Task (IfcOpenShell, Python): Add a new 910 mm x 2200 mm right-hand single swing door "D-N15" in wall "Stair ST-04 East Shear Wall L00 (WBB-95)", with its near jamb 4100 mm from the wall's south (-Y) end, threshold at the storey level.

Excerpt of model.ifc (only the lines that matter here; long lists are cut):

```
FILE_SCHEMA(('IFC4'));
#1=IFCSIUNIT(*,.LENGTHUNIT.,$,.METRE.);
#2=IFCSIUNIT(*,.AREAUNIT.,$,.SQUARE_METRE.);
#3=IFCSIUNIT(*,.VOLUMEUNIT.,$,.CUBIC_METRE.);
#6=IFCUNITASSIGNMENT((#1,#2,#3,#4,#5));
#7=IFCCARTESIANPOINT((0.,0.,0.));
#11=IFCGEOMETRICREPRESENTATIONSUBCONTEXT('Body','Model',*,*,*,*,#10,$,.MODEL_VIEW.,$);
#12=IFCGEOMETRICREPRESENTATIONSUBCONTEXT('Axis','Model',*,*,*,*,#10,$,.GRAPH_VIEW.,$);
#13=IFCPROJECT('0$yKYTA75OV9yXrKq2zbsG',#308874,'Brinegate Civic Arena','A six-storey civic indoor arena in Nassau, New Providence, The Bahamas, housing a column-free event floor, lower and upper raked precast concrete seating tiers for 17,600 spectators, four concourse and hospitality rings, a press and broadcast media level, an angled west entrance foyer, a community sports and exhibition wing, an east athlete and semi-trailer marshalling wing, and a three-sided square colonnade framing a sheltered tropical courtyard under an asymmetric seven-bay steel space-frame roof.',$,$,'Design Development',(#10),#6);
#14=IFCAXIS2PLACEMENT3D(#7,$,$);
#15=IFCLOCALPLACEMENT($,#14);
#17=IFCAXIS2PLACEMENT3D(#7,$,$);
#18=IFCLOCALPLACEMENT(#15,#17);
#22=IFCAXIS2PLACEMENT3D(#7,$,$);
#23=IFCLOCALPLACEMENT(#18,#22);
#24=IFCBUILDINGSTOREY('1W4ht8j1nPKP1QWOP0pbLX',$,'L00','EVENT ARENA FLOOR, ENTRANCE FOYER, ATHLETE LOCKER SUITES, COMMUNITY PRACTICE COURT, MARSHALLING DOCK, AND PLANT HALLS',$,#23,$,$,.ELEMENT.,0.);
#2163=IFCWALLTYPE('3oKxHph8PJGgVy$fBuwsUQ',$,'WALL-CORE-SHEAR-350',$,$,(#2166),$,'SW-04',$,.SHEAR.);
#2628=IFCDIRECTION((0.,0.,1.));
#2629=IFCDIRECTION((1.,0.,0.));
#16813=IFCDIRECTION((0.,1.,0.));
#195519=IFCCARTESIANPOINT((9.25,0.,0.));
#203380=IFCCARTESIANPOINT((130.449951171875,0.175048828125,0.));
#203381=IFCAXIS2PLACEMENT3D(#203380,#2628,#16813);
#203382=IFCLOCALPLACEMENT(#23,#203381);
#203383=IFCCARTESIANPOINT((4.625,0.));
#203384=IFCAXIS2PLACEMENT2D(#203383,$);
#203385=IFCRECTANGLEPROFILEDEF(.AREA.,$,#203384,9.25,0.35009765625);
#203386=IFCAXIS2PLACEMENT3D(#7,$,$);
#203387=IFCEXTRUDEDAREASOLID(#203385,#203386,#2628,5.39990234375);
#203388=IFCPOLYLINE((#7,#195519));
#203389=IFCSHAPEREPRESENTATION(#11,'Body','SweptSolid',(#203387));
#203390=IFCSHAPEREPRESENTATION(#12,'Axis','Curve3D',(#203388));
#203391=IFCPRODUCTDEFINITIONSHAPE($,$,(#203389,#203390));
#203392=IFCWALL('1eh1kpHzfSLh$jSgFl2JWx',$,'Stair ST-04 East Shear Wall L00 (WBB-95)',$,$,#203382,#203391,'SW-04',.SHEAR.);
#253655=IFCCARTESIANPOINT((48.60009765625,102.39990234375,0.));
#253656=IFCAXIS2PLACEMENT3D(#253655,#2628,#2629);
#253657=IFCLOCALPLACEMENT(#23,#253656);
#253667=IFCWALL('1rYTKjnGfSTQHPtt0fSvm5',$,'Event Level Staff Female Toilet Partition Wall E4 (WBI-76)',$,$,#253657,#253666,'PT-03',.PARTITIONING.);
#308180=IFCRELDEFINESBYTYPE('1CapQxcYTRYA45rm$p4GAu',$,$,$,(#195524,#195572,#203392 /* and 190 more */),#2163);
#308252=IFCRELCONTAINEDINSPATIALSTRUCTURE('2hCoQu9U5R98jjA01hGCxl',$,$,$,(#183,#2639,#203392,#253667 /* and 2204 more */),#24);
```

```python
import numpy as np
import ifcopenshell
import ifcopenshell.api.feature
import ifcopenshell.api.geometry
import ifcopenshell.api.root
import ifcopenshell.api.spatial
import ifcopenshell.geom
import ifcopenshell.util.element
import ifcopenshell.util.placement
import ifcopenshell.util.representation
import ifcopenshell.util.shape
import ifcopenshell.util.unit

model = ifcopenshell.open("model.ifc")
unit_scale = ifcopenshell.util.unit.calculate_unit_scale(model)
settings = ifcopenshell.geom.settings()


def volume(element):
    """Net volume in cubic metres, openings subtracted."""
    shape = ifcopenshell.geom.create_shape(settings, element)
    return ifcopenshell.util.shape.get_volume(shape.geometry)


wall = model.by_guid("1eh1kpHzfSLh$jSgFl2JWx")
storey = ifcopenshell.util.element.get_container(wall, ifc_class="IfcBuildingStorey")
context = ifcopenshell.util.representation.get_context(model, "Model", "Body", "MODEL_VIEW")
before = volume(wall)

width, height, from_end, sill = 0.91, 2.2, 4.1, 0.0  # metres

# The wall runs along its own X axis, and the end named is its -X end.
wall_shape = ifcopenshell.geom.create_shape(settings, wall)
x, y, z = ifcopenshell.util.shape.get_vertices(wall_shape.geometry).T
start = x.min() + from_end
face, thickness = float(y.min()), float(y.max() - y.min())
wall_matrix = ifcopenshell.util.placement.get_local_placement(wall.ObjectPlacement)
level = ifcopenshell.util.placement.get_local_placement(storey.ObjectPlacement)[2, 3]


def in_wall(x, y):
    """Placement at x, y metres in the wall's axes, at sill height."""
    matrix = wall_matrix.copy()
    matrix[:, 3] = wall_matrix @ np.array([x / unit_scale, y / unit_scale, 0.0, 1.0])
    matrix[2, 3] = level + sill / unit_scale
    return matrix


# Opening: a box that overshoots both wall faces by 50 mm.
opening = ifcopenshell.api.root.create_entity(model, ifc_class="IfcOpeningElement", predefined_type="OPENING")
box = ifcopenshell.api.geometry.add_wall_representation(
    model, context=context, length=width, height=height, thickness=thickness + 0.1
)
ifcopenshell.api.geometry.assign_representation(model, product=opening, representation=box)
ifcopenshell.api.geometry.edit_object_placement(model, product=opening, matrix=in_wall(start, face - 0.05), is_si=False)
ifcopenshell.api.feature.add_feature(model, feature=opening, element=wall)

door = ifcopenshell.api.root.create_entity(model, ifc_class="IfcDoor", name="D-N15", predefined_type="DOOR")
door.OverallWidth, door.OverallHeight = width / unit_scale, height / unit_scale
door.OperationType = "SINGLE_SWING_RIGHT"
body = ifcopenshell.api.geometry.add_door_representation(
    model,
    context=context,
    overall_width=door.OverallWidth,
    overall_height=door.OverallHeight,
    operation_type="SINGLE_SWING_RIGHT",
    lining_properties={"LiningDepth": thickness / unit_scale, "ThresholdDepth": thickness / unit_scale},
)
ifcopenshell.api.geometry.assign_representation(model, product=door, representation=body)
ifcopenshell.api.spatial.assign_container(model, products=[door], relating_structure=storey)
ifcopenshell.api.feature.add_filling(model, opening=opening, element=door)

# The lining spans the wall, so the door starts at the wall face.
ifcopenshell.api.geometry.edit_object_placement(model, product=door, matrix=in_wall(start, face), is_si=False)

after = volume(wall)

print(f"wall volume {before:.3f} -> {after:.3f} m3")

model.write("model_edited.ifc")
```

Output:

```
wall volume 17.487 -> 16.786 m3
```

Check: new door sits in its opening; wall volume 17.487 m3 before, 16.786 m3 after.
